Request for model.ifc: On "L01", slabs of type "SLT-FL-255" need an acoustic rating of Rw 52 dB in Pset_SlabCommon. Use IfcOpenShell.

First a look at what the model holds.

```python
import ifcopenshell
import ifcopenshell.util.element

model = ifcopenshell.open("model.ifc")
print(model.schema)
storey = next(s for s in model.by_type("IfcBuildingStorey") if s.Name == "L01")
slabs = [e for e in ifcopenshell.util.element.get_decomposition(storey) if e.is_a("IfcSlab")]
seen = {}
for e in slabs:
    element_type = ifcopenshell.util.element.get_type(e)
    key = (element_type.Name if element_type != e and element_type else None, ifcopenshell.util.element.get_pset(e, "Pset_SlabCommon", "AcousticRating"))
    seen[key] = seen.get(key, 0) + 1
for (name, value), count in sorted(seen.items(), key=str):
    print(count, "x", name, "|", value)
```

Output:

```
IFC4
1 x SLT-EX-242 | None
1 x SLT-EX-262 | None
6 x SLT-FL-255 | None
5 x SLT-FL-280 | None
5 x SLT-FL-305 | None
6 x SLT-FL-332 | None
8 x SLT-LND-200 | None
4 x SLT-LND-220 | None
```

```python
import ifcopenshell
import ifcopenshell.api.pset
import ifcopenshell.util.element

model = ifcopenshell.open("model.ifc")

storey = next(s for s in model.by_type("IfcBuildingStorey") if s.Name == "L01")
slabs = [e for e in ifcopenshell.util.element.get_decomposition(storey) if e.is_a("IfcSlab")]

count = 0
for e in slabs:
    element_type = ifcopenshell.util.element.get_type(e)
    if element_type in (None, e) or element_type.Name != "SLT-FL-255":
        continue
    # add_pset returns the element's existing set when there is one.
    pset = ifcopenshell.api.pset.add_pset(model, product=e, name="Pset_SlabCommon")
    ifcopenshell.api.pset.edit_pset(model, pset=pset, properties={"AcousticRating": "Rw 52 dB"})
    count += 1

print(count, "slabs updated")

model.write("model_v2.ifc")
```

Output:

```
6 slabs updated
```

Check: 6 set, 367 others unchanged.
